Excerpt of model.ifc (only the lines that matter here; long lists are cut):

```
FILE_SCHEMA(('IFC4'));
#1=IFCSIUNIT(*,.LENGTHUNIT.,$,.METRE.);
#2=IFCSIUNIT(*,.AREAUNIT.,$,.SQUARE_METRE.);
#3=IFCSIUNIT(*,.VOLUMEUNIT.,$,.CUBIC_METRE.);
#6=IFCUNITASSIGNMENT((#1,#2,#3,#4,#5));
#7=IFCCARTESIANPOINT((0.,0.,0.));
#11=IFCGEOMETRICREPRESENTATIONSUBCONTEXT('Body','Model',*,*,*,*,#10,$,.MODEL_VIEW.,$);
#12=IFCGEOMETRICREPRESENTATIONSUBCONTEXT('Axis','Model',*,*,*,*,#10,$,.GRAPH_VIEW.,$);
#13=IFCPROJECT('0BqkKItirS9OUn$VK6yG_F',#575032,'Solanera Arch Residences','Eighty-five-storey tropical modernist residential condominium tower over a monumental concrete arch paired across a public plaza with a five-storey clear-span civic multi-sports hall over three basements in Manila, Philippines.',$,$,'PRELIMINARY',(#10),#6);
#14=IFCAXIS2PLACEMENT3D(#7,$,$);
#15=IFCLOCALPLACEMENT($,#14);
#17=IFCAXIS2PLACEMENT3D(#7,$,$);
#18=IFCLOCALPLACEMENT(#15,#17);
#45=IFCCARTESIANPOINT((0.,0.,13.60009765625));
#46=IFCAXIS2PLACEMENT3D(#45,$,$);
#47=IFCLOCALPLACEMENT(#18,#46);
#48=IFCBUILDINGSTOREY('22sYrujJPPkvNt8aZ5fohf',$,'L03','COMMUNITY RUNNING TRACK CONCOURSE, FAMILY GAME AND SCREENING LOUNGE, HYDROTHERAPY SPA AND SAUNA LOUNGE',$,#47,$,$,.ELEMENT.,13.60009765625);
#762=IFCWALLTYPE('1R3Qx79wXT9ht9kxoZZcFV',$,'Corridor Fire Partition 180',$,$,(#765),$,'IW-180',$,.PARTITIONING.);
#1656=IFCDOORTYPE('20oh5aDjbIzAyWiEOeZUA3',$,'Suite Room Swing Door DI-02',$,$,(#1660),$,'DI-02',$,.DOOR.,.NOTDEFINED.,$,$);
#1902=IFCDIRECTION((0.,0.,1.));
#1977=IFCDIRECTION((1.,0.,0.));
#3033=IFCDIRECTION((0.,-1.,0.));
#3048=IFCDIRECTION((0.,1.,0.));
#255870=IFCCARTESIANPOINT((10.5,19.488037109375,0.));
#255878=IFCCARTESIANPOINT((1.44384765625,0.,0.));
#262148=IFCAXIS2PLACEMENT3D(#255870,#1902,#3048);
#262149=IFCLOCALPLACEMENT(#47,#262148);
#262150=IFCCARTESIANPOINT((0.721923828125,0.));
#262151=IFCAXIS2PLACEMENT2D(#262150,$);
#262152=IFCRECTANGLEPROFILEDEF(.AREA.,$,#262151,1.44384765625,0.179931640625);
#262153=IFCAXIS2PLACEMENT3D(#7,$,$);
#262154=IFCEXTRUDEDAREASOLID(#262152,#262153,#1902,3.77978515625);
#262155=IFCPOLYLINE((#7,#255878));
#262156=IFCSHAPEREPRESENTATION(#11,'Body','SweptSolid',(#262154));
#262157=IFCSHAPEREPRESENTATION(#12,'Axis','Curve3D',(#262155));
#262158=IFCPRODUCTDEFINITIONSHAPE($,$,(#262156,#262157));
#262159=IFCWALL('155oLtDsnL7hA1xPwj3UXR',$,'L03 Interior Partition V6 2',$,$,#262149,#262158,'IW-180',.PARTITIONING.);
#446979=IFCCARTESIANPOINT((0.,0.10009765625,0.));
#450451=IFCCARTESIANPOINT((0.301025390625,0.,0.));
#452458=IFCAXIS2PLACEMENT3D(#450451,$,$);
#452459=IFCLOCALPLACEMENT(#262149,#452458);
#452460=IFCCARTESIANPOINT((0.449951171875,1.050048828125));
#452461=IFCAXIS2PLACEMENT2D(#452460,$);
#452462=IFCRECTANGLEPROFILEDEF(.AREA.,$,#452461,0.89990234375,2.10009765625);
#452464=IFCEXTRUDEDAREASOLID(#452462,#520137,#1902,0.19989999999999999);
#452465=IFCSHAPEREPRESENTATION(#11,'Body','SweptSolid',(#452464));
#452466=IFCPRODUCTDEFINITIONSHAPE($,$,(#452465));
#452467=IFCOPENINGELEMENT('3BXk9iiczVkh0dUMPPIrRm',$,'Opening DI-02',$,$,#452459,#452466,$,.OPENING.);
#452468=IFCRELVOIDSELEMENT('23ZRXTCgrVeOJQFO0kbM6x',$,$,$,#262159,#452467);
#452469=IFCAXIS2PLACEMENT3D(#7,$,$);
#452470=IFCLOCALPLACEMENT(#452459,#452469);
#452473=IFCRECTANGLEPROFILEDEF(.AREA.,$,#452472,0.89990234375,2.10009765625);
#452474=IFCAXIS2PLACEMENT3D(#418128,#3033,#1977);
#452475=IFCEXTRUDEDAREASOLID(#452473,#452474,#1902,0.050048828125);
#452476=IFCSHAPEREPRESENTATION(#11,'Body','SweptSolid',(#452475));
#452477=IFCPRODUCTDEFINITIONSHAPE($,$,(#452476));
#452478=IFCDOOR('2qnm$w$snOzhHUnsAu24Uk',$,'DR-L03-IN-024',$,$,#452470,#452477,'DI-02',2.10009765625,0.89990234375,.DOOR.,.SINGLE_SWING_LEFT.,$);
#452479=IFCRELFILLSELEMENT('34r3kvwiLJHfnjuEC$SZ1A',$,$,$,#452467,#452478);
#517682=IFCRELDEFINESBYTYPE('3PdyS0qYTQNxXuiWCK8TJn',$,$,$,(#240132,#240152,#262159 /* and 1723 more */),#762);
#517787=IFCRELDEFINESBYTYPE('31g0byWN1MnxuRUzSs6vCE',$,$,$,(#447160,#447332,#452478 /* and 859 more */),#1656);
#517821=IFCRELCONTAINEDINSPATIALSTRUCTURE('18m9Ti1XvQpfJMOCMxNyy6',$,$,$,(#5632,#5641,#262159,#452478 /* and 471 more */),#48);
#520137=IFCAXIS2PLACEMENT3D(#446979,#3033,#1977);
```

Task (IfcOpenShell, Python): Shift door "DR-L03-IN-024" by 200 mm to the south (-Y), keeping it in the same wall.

```python
import ifcopenshell
import ifcopenshell.api.geometry
import ifcopenshell.util.placement
import ifcopenshell.util.unit

model = ifcopenshell.open("model.ifc")
unit_scale = ifcopenshell.util.unit.calculate_unit_scale(model)

door = model.by_id(452478)
opening = door.FillsVoids[0].RelatingOpeningElement
wall = opening.VoidsElements[0].RelatingBuildingElement

wall_matrix = ifcopenshell.util.placement.get_local_placement(wall.ObjectPlacement)
shift = wall_matrix[:3, 0] * -0.2 / unit_scale
before = ifcopenshell.util.placement.get_local_placement(door.ObjectPlacement)[:3, 3].copy()

# The door is placed relative to its opening, so it follows when the opening moves.
matrix = ifcopenshell.util.placement.get_local_placement(opening.ObjectPlacement)
matrix[:3, 3] += shift
ifcopenshell.api.geometry.edit_object_placement(
    model, product=opening, matrix=matrix, is_si=False, should_transform_children=True
)

after = ifcopenshell.util.placement.get_local_placement(door.ObjectPlacement)[:3, 3]
print("door moved by", (after - before).round(3) + 0.0)

model.write("model-out.ifc")
```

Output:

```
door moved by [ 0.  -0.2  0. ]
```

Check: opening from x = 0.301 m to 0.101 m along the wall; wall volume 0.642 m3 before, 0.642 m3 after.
